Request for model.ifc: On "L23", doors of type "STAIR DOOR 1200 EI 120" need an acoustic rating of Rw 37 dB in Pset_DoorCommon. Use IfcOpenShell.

First a look at what the model holds.

```python
import ifcopenshell
import ifcopenshell.util.element

model = ifcopenshell.open("model.ifc")
print(model.schema)
storey = next(s for s in model.by_type("IfcBuildingStorey") if s.Name == "L23")
doors = [e for e in ifcopenshell.util.element.get_decomposition(storey) if e.is_a("IfcDoor")]
seen = {}
for e in doors:
    element_type = ifcopenshell.util.element.get_type(e)
    key = (element_type.Name if element_type != e and element_type else None, ifcopenshell.util.element.get_pset(e, "Pset_DoorCommon", "AcousticRating"))
    seen[key] = seen.get(key, 0) + 1
for (name, value), count in sorted(seen.items(), key=str):
    print(count, "x", name, "|", value)
```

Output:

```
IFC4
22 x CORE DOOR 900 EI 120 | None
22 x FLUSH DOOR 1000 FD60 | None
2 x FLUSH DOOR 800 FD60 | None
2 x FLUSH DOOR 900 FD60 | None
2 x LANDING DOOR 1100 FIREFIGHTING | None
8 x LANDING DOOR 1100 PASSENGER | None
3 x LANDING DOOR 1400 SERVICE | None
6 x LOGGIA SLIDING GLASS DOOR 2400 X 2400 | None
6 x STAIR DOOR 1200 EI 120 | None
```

```python
import ifcopenshell
import ifcopenshell.api.pset
import ifcopenshell.util.element

model = ifcopenshell.open("model.ifc")

storey = next(s for s in model.by_type("IfcBuildingStorey") if s.Name == "L23")
doors = [e for e in ifcopenshell.util.element.get_decomposition(storey) if e.is_a("IfcDoor")]

count = 0
for e in doors:
    element_type = ifcopenshell.util.element.get_type(e)
    if element_type in (None, e) or element_type.Name != "STAIR DOOR 1200 EI 120":
        continue
    found = ifcopenshell.util.element.get_pset(e, "Pset_DoorCommon", should_inherit=False)
    if found:
        pset = model.by_id(found["id"])
        if len(ifcopenshell.util.element.get_elements_by_pset(pset)) > 1:
            pset = ifcopenshell.api.pset.unshare_pset(model, products=[e], pset=pset)[0]
    else:
        pset = ifcopenshell.api.pset.add_pset(model, product=e, name="Pset_DoorCommon")
    ifcopenshell.api.pset.edit_pset(model, pset=pset, properties={"AcousticRating": "Rw 37 dB"})
    count += 1

print(count, "doors updated")

model.write("model_edited.ifc")
```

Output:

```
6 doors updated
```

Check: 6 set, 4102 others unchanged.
